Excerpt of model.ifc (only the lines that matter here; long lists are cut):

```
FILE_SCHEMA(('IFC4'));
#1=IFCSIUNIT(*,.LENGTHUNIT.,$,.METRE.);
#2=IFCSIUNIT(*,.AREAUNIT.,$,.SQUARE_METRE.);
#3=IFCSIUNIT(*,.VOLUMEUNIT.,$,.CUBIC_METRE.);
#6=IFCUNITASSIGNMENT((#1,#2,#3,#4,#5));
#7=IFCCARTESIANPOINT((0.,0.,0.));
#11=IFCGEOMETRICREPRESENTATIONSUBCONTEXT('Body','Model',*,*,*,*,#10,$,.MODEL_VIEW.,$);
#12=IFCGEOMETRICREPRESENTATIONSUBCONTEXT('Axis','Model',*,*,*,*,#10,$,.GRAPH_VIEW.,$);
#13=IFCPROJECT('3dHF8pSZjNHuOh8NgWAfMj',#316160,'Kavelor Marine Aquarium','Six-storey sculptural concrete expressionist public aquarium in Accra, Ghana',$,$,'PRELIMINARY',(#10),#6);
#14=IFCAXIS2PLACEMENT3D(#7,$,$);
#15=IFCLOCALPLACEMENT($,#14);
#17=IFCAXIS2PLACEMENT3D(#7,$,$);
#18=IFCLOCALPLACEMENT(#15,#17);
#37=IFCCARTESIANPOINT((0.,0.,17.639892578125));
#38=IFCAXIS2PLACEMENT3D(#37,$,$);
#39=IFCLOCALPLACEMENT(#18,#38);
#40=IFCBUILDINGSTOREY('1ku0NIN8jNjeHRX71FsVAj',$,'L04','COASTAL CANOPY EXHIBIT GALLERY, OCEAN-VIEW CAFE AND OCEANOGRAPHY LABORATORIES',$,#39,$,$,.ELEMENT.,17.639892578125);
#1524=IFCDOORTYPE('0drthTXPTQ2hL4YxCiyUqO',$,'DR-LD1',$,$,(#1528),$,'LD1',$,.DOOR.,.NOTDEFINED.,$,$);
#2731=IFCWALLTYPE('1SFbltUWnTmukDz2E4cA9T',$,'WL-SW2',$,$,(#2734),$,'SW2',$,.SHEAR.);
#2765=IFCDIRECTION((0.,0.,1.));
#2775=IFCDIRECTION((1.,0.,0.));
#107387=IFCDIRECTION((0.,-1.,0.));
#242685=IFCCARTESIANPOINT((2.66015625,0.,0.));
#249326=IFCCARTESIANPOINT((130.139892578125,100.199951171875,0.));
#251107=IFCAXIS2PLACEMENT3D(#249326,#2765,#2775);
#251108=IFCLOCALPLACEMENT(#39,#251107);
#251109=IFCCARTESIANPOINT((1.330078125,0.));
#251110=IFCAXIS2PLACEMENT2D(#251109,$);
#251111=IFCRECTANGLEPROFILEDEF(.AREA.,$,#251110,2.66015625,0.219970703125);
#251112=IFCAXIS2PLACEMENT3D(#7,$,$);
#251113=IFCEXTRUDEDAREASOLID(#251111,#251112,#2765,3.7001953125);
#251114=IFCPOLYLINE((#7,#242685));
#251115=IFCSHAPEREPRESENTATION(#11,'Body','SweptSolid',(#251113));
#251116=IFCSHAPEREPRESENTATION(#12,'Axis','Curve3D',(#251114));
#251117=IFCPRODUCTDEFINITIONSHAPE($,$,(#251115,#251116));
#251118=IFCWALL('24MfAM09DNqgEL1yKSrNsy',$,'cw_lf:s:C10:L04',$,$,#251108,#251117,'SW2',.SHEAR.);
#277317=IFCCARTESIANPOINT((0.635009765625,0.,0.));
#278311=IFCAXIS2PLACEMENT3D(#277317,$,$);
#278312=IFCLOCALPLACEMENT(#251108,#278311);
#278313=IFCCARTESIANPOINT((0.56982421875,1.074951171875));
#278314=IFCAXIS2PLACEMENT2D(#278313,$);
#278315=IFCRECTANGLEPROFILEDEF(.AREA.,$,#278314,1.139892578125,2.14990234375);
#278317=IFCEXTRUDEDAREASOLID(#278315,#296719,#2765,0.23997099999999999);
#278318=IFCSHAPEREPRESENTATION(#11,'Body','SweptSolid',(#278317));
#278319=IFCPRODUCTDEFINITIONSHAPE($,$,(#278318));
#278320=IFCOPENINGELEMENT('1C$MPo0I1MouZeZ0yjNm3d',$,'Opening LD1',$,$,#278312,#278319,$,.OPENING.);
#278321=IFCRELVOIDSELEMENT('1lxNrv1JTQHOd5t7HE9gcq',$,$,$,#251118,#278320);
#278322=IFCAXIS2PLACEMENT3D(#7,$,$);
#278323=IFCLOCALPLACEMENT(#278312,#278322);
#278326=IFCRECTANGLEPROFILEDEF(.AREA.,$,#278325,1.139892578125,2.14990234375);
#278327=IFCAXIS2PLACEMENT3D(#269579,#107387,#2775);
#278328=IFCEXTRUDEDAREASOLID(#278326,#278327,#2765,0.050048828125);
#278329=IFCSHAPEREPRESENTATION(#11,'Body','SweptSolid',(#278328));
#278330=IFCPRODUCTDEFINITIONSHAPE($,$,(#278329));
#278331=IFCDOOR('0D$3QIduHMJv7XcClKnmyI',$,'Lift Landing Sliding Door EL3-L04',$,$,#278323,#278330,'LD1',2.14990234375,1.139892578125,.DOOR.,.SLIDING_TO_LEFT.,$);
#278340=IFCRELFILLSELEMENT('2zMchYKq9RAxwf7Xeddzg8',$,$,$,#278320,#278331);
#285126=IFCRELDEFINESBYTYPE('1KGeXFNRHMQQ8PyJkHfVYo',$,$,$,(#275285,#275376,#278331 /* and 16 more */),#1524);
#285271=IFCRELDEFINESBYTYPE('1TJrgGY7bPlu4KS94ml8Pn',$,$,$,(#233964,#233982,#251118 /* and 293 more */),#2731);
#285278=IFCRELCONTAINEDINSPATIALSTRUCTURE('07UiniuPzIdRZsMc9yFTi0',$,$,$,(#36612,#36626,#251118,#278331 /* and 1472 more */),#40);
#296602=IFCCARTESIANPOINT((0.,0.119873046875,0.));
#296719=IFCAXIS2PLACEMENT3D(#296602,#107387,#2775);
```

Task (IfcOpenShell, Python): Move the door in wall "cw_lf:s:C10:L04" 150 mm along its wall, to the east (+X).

```python
import ifcopenshell
import ifcopenshell.api.geometry
import ifcopenshell.util.placement

model = ifcopenshell.open("model.ifc")

door = model.by_guid("0D$3QIduHMJv7XcClKnmyI")
opening = door.FillsVoids[0].RelatingOpeningElement
wall = opening.VoidsElements[0].RelatingBuildingElement

wall_matrix = ifcopenshell.util.placement.get_local_placement(wall.ObjectPlacement)
shift = wall_matrix[:3, 0] * 0.15
before = ifcopenshell.util.placement.get_local_placement(door.ObjectPlacement)[:3, 3].copy()

# The door is placed relative to its opening, so it follows when the opening moves.
matrix = ifcopenshell.util.placement.get_local_placement(opening.ObjectPlacement)
matrix[:3, 3] += shift
ifcopenshell.api.geometry.edit_object_placement(
    model, product=opening, matrix=matrix, is_si=False, should_transform_children=True
)

after = ifcopenshell.util.placement.get_local_placement(door.ObjectPlacement)[:3, 3]
print("door moved by", (after - before).round(3) + 0.0)

model.write("model-out.ifc")
```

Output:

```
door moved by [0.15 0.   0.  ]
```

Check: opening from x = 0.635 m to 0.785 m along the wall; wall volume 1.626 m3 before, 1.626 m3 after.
